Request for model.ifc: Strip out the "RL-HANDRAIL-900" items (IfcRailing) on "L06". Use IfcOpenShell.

First a look at what the model holds.

```python
import ifcopenshell
import ifcopenshell.util.element

model = ifcopenshell.open("model.ifc")
print(model.schema)
storey = next(s for s in model.by_type("IfcBuildingStorey") if s.Name == "L06")
railings = [e for e in ifcopenshell.util.element.get_decomposition(storey) if e.is_a("IfcRailing")]
seen = {}
for e in railings:
    element_type = ifcopenshell.util.element.get_type(e)
    name = element_type.Name if element_type not in (None, e) else None
    seen[name] = seen.get(name, 0) + 1
for name, count in sorted(seen.items(), key=str):
    print(count, "x", name)
```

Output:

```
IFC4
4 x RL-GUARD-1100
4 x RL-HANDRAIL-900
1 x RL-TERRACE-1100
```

```python
import ifcopenshell
import ifcopenshell.api.root
import ifcopenshell.util.element

model = ifcopenshell.open("model.ifc")

storey = next(s for s in model.by_type("IfcBuildingStorey") if s.Name == "L06")
railings = [e for e in ifcopenshell.util.element.get_decomposition(storey) if e.is_a("IfcRailing")]
targets = [e for e in railings if (t := ifcopenshell.util.element.get_type(e)) not in (None, e) and t.Name == "RL-HANDRAIL-900"]

for e in targets:
    ifcopenshell.api.root.remove_product(model, product=e)
print(len(targets), "removed")

model.write("model-out.ifc")
```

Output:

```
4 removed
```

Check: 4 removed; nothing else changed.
